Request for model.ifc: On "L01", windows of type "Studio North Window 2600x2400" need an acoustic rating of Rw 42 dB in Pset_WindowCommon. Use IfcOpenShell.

First a look at what the model holds.

```python
import ifcopenshell
import ifcopenshell.util.element

model = ifcopenshell.open("model.ifc")
print(model.schema)
storey = next(s for s in model.by_type("IfcBuildingStorey") if s.Name == "L01")
windows = [e for e in ifcopenshell.util.element.get_decomposition(storey) if e.is_a("IfcWindow")]
seen = {}
for e in windows:
    element_type = ifcopenshell.util.element.get_type(e)
    key = (element_type.Name if element_type != e and element_type else None, ifcopenshell.util.element.get_pset(e, "Pset_WindowCommon", "AcousticRating"))
    seen[key] = seen.get(key, 0) + 1
for (name, value), count in sorted(seen.items(), key=str):
    print(count, "x", name, "|", value)
```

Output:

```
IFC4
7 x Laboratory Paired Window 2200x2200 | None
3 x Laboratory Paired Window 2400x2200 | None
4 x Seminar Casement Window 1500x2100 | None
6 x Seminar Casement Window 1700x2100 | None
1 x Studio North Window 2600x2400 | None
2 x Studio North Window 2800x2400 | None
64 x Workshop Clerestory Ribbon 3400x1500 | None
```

```python
import ifcopenshell
import ifcopenshell.api.pset
import ifcopenshell.util.element

model = ifcopenshell.open("model.ifc")

storey = next(s for s in model.by_type("IfcBuildingStorey") if s.Name == "L01")
windows = [e for e in ifcopenshell.util.element.get_decomposition(storey) if e.is_a("IfcWindow")]

count = 0
for e in windows:
    element_type = ifcopenshell.util.element.get_type(e)
    if element_type in (None, e) or element_type.Name != "Studio North Window 2600x2400":
        continue
    # add_pset returns the element's existing set when there is one.
    pset = ifcopenshell.api.pset.add_pset(model, product=e, name="Pset_WindowCommon")
    ifcopenshell.api.pset.edit_pset(model, pset=pset, properties={"AcousticRating": "Rw 42 dB"})
    count += 1

print(count, "windows updated")

model.write("model_v2.ifc")
```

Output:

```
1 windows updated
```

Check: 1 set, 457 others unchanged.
